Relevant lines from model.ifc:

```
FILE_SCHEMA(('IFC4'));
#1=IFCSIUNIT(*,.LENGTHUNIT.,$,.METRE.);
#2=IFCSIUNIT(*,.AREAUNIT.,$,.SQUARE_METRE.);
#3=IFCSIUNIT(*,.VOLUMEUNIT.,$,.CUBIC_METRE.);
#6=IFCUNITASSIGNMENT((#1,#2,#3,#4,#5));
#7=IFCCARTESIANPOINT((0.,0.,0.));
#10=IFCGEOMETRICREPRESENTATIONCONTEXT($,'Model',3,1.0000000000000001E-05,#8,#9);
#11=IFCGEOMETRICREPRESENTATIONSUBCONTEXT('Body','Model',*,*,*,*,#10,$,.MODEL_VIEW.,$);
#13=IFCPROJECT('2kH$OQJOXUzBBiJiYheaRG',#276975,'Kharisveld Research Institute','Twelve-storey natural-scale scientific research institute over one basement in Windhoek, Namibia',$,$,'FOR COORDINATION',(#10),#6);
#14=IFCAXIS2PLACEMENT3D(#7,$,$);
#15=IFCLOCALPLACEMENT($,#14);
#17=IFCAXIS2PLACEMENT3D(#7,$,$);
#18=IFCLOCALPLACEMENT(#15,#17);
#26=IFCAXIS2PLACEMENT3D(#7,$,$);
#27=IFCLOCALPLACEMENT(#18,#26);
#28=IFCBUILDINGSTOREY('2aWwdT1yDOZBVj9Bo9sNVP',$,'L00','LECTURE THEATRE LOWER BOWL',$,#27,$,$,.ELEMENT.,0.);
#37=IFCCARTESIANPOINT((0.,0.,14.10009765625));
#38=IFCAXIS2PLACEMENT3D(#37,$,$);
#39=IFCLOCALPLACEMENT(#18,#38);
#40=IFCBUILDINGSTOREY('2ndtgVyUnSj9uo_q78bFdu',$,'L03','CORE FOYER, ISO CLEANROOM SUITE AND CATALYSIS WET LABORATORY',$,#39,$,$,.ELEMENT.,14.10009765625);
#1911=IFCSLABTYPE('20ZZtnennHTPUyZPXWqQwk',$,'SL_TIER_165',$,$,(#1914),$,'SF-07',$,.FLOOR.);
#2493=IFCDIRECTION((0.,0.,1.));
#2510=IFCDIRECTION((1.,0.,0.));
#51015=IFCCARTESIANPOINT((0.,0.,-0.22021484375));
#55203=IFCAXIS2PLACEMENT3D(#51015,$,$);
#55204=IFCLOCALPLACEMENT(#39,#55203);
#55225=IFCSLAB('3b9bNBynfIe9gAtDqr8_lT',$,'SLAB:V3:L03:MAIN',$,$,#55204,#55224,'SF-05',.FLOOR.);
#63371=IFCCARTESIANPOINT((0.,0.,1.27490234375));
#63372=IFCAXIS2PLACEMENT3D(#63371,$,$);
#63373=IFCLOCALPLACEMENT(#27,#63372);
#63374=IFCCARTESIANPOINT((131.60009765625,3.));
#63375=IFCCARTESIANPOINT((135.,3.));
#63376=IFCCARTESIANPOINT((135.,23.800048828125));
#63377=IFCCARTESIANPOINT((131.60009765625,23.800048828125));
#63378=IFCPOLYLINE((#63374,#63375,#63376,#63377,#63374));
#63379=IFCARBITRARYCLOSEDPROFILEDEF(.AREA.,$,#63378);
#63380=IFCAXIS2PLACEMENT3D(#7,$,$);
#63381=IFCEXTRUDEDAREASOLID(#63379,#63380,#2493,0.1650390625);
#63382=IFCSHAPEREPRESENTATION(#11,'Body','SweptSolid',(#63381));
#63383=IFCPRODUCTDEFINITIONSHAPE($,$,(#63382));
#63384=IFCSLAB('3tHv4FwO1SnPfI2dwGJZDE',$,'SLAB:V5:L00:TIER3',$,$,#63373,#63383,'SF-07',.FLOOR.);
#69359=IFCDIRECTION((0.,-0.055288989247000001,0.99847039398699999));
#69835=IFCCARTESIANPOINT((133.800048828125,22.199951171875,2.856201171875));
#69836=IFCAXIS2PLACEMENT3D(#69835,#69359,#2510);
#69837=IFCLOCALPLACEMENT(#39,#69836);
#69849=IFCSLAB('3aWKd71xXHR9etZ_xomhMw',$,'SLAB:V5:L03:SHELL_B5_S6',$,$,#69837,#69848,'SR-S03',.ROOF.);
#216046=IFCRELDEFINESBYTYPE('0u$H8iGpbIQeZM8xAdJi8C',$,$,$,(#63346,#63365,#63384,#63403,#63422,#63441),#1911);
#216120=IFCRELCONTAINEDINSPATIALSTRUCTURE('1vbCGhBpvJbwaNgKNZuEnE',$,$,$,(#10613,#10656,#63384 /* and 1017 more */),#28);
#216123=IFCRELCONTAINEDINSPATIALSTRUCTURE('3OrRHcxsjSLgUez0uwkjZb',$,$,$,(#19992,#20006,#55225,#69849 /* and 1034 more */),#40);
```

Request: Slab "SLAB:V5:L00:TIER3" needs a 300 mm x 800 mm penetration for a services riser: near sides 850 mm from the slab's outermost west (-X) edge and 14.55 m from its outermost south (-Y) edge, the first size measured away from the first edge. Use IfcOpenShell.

```python
import numpy as np
import ifcopenshell
import ifcopenshell.api.feature
import ifcopenshell.api.geometry
import ifcopenshell.api.root
import ifcopenshell.geom
import ifcopenshell.util.placement
import ifcopenshell.util.representation
import ifcopenshell.util.shape
import ifcopenshell.util.unit

model = ifcopenshell.open("model.ifc")
unit_scale = ifcopenshell.util.unit.calculate_unit_scale(model)
settings = ifcopenshell.geom.settings()


def volume(element):
    """Net volume in cubic metres, openings subtracted."""
    shape = ifcopenshell.geom.create_shape(settings, element)
    return ifcopenshell.util.shape.get_volume(shape.geometry)


slab = model.by_id(63384)
before = volume(slab)

# Extent in the slab's own axes, in metres. The edges named are its -X and -Y sides.
slab_shape = ifcopenshell.geom.create_shape(settings, slab)
vertices = ifcopenshell.util.shape.get_vertices(slab_shape.geometry)
x_min, y_min, bottom = vertices.min(axis=0)
top = vertices[:, 2].max()

opening = ifcopenshell.api.root.create_entity(model, ifc_class="IfcOpeningElement", name="Services riser opening", predefined_type="OPENING")
context = ifcopenshell.util.representation.get_context(model, "Model", "Body", "MODEL_VIEW")
width, depth = 0.3, 0.8
outline = [(0.0, 0.0), (width, 0.0), (width, depth), (0.0, depth), (0.0, 0.0)]
# Overshoot both faces by 50 mm so the cut is clean.
shape = ifcopenshell.api.geometry.add_slab_representation(
    model, context=context, depth=top - bottom + 0.1, polyline=outline
)
ifcopenshell.api.geometry.assign_representation(model, product=opening, representation=shape)

matrix = ifcopenshell.util.placement.get_local_placement(slab.ObjectPlacement)
matrix[:, 3] = matrix @ np.append(np.array([x_min + 0.85, y_min + 14.55, bottom - 0.05]) / unit_scale, 1.0)
ifcopenshell.api.geometry.edit_object_placement(model, product=opening, matrix=matrix, is_si=False)
ifcopenshell.api.feature.add_feature(model, feature=opening, element=slab)

after = volume(slab)

print(f"slab volume {before:.3f} -> {after:.3f} m3")

model.write("model_v2.ifc")
```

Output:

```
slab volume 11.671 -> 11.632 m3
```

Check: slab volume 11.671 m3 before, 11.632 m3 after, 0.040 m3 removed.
